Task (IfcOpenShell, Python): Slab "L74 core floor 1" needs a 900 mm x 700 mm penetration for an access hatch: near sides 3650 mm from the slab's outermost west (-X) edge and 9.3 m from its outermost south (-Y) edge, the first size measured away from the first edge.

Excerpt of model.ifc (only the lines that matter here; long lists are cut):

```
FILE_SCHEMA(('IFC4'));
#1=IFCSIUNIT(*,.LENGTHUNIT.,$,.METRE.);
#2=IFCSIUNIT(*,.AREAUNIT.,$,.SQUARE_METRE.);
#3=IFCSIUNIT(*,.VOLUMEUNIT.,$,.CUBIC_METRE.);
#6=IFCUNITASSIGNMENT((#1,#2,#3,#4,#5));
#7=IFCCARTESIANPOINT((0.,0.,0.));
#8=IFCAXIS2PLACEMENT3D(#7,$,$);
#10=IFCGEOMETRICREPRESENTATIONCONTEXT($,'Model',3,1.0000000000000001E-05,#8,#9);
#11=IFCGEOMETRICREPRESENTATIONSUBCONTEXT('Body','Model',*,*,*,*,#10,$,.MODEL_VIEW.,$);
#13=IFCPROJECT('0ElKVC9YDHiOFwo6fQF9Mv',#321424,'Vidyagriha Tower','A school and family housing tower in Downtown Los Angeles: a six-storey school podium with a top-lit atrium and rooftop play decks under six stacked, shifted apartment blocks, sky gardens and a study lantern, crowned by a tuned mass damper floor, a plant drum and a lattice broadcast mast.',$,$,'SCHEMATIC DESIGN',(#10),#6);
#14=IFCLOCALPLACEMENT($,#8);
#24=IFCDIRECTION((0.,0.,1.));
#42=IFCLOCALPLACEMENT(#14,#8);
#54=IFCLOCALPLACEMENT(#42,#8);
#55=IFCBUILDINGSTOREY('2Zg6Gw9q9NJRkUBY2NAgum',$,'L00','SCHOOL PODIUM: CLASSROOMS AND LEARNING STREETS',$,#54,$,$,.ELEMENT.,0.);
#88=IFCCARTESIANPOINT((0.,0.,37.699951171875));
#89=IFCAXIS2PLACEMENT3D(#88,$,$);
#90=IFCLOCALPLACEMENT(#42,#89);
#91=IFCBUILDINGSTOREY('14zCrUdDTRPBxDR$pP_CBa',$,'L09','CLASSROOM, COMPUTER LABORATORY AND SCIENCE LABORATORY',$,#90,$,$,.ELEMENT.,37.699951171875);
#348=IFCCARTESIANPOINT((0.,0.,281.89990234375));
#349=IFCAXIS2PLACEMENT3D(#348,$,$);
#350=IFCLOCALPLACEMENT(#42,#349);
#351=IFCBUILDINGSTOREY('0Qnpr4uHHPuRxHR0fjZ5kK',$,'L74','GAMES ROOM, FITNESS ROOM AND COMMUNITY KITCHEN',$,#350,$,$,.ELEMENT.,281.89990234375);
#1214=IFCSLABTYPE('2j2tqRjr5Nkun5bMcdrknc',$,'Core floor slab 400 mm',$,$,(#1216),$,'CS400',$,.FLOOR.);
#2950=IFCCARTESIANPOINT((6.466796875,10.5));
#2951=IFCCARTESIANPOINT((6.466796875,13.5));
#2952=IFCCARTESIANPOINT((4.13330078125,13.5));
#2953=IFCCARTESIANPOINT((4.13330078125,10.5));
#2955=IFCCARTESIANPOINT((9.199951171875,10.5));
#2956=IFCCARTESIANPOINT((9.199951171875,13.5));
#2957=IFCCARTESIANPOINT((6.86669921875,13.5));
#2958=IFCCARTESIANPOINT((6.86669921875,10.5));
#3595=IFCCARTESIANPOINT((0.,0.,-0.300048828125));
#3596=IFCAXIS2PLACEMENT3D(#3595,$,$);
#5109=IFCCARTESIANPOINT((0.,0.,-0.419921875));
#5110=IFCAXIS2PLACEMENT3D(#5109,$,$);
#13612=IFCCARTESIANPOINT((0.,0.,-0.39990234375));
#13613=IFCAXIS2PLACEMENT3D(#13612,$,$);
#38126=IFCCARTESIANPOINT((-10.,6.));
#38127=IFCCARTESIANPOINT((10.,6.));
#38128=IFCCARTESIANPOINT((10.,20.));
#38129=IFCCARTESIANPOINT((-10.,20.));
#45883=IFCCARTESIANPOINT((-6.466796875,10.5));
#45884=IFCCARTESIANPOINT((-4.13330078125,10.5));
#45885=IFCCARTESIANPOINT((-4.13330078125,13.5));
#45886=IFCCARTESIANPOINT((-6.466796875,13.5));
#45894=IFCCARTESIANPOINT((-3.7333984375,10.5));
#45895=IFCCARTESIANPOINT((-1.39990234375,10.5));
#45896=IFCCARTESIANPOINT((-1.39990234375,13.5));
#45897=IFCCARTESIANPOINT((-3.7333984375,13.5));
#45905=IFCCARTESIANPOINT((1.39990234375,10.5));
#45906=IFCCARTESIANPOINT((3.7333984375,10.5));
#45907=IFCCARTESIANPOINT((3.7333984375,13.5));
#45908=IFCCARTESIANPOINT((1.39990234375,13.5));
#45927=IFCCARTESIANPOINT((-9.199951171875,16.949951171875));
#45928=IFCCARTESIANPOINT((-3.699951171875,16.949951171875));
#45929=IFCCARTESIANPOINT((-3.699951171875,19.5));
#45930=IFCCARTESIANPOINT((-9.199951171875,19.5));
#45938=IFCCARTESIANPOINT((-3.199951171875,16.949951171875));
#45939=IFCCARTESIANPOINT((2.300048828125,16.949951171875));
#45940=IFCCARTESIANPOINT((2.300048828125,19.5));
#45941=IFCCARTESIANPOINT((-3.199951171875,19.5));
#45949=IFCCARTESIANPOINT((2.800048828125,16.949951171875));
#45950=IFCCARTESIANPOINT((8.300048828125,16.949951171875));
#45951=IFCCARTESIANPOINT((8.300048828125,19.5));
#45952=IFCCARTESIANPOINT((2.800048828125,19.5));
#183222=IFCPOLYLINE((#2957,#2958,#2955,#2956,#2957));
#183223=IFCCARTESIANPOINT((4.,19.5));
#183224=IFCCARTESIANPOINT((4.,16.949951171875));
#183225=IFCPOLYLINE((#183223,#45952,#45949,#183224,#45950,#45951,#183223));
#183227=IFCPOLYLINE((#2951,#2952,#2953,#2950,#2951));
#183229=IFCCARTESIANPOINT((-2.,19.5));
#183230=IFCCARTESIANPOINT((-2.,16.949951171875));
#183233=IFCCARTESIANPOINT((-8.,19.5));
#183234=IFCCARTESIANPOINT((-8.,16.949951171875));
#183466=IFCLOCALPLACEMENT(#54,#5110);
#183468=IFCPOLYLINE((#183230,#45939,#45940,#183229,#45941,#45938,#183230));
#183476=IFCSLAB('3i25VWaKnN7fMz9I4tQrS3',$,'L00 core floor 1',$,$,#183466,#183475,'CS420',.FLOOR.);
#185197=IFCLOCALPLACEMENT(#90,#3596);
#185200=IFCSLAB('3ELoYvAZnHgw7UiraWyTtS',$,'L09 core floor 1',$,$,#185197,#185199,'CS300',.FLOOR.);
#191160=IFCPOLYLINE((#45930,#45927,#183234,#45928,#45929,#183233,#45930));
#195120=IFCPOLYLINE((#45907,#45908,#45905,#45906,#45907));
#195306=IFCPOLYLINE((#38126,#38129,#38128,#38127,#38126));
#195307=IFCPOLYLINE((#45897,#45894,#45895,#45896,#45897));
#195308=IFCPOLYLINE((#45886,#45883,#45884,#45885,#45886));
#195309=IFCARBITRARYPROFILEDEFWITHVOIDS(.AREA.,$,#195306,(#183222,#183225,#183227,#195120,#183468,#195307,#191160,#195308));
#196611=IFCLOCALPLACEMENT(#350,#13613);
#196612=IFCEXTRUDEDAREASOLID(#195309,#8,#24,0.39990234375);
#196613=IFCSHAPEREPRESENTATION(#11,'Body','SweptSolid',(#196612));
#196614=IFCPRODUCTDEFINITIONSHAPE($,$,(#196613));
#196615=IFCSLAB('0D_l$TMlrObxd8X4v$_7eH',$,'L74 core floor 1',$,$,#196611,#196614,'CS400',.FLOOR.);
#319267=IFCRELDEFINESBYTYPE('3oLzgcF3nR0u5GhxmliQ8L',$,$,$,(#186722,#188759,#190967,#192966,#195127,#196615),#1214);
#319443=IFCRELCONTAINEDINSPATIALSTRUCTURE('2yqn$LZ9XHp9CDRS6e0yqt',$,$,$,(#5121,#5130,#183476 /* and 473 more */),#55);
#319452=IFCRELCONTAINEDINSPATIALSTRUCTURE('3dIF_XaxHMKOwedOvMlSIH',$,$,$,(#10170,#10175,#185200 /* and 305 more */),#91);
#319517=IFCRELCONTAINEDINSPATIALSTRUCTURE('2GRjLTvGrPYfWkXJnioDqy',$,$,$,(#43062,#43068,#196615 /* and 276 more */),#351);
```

```python
import numpy as np
import ifcopenshell
import ifcopenshell.api.feature
import ifcopenshell.api.geometry
import ifcopenshell.api.root
import ifcopenshell.geom
import ifcopenshell.util.placement
import ifcopenshell.util.representation
import ifcopenshell.util.shape
import ifcopenshell.util.unit

model = ifcopenshell.open("model.ifc")
unit_scale = ifcopenshell.util.unit.calculate_unit_scale(model)
settings = ifcopenshell.geom.settings()


def volume(element):
    """Net volume in cubic metres, openings subtracted."""
    shape = ifcopenshell.geom.create_shape(settings, element)
    return ifcopenshell.util.shape.get_volume(shape.geometry)


slab = model.by_guid("0D_l$TMlrObxd8X4v$_7eH")
before = volume(slab)

# Extent in the slab's own axes, in metres. The edges named are its -X and -Y sides.
slab_shape = ifcopenshell.geom.create_shape(settings, slab)
vertices = ifcopenshell.util.shape.get_vertices(slab_shape.geometry)
x_min, y_min, bottom = vertices.min(axis=0)
top = vertices[:, 2].max()

opening = ifcopenshell.api.root.create_entity(model, ifc_class="IfcOpeningElement", name="Access hatch opening", predefined_type="OPENING")
context = ifcopenshell.util.representation.get_context(model, "Model", "Body", "MODEL_VIEW")
width, depth = 0.9, 0.7
outline = [(0.0, 0.0), (width, 0.0), (width, depth), (0.0, depth), (0.0, 0.0)]
# Overshoot both faces by 50 mm so the cut is clean.
shape = ifcopenshell.api.geometry.add_slab_representation(
    model, context=context, depth=top - bottom + 0.1, polyline=outline
)
ifcopenshell.api.geometry.assign_representation(model, product=opening, representation=shape)

matrix = ifcopenshell.util.placement.get_local_placement(slab.ObjectPlacement)
matrix[:, 3] = matrix @ np.append(np.array([x_min + 3.65, y_min + 9.3, bottom - 0.05]) / unit_scale, 1.0)
ifcopenshell.api.geometry.edit_object_placement(model, product=opening, matrix=matrix, is_si=False)
ifcopenshell.api.feature.add_feature(model, feature=opening, element=slab)

after = volume(slab)

print(f"slab volume {before:.3f} -> {after:.3f} m3")

model.write("model_v2.ifc")
```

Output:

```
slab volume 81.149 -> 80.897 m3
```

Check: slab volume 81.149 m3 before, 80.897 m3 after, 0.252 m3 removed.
